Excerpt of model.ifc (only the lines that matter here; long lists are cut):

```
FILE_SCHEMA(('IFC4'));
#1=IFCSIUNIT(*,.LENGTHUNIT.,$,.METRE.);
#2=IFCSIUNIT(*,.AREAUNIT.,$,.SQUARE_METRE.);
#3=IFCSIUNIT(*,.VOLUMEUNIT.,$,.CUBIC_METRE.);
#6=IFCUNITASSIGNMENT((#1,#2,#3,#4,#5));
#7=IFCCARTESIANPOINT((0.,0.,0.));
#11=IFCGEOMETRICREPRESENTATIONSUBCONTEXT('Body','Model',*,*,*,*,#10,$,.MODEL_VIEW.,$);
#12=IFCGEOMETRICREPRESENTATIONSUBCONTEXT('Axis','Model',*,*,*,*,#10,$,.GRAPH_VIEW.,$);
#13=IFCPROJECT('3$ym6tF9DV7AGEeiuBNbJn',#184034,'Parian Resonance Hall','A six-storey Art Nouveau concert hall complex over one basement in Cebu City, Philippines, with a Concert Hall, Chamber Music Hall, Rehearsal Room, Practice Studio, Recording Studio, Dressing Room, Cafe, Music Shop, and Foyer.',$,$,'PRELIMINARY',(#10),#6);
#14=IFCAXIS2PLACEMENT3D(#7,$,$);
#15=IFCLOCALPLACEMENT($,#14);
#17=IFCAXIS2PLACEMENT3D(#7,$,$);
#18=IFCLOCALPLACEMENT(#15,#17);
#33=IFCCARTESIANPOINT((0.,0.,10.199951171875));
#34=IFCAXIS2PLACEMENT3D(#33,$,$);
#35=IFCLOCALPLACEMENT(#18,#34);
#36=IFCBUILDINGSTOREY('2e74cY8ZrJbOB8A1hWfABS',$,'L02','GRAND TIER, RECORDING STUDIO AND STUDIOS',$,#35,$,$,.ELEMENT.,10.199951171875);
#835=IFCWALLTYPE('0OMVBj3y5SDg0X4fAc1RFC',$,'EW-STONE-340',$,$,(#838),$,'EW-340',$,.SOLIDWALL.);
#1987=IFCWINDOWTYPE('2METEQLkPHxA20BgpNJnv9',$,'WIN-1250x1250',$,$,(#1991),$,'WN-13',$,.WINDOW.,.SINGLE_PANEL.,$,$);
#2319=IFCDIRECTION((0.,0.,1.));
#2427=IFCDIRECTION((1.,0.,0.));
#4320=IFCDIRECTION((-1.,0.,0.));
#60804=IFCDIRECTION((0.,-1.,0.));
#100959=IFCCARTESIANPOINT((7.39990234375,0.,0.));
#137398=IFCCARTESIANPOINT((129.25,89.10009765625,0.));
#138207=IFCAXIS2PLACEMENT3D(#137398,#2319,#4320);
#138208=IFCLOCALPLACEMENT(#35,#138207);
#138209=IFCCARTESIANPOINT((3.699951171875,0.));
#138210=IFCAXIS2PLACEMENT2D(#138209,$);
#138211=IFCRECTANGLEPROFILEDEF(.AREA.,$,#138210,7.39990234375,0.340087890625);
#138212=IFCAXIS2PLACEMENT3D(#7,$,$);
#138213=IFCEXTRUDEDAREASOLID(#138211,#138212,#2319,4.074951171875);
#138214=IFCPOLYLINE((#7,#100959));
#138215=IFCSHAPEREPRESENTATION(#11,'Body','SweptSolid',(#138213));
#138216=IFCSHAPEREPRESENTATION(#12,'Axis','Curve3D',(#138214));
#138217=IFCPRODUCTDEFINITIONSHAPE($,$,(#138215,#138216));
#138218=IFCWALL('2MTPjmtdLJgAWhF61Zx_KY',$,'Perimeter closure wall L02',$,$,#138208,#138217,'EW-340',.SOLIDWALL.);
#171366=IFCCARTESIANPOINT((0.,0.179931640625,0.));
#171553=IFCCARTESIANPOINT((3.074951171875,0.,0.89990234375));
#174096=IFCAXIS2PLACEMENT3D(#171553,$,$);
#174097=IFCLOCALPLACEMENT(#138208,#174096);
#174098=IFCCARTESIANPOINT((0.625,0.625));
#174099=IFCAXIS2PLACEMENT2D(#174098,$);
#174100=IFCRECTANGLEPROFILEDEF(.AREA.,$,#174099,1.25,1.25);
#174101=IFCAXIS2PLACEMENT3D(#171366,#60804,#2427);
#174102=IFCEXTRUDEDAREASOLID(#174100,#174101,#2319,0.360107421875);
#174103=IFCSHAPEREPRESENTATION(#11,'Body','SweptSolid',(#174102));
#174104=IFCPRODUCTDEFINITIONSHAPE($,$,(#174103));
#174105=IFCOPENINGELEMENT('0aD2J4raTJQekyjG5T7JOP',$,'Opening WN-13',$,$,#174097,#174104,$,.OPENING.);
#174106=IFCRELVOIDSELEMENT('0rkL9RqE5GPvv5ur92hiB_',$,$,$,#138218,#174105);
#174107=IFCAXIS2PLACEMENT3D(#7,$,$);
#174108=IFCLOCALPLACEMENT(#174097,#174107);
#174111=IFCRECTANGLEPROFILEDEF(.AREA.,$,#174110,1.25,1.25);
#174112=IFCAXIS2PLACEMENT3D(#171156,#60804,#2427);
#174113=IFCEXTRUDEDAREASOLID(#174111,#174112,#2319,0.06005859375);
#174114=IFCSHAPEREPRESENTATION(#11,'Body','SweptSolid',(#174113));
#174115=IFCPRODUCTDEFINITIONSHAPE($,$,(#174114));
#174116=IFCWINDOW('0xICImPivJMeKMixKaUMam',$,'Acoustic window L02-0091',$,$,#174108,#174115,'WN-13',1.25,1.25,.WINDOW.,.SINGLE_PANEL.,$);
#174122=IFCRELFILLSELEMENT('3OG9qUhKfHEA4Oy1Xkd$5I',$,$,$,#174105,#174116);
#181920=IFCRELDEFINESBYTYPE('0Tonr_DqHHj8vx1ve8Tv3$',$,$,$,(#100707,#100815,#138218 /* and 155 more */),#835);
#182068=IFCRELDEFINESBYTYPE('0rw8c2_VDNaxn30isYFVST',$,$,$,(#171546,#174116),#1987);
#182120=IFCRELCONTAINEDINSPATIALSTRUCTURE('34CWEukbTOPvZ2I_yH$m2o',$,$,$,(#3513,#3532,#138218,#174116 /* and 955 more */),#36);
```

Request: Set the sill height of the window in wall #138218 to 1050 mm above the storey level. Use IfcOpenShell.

```python
import numpy as np
import ifcopenshell
import ifcopenshell.api.geometry
import ifcopenshell.geom
import ifcopenshell.util.element
import ifcopenshell.util.placement
import ifcopenshell.util.shape
import ifcopenshell.util.unit

model = ifcopenshell.open("model.ifc")
unit_scale = ifcopenshell.util.unit.calculate_unit_scale(model)

window = model.by_guid("0xICImPivJMeKMixKaUMam")
opening = window.FillsVoids[0].RelatingOpeningElement
storey = ifcopenshell.util.element.get_container(window, ifc_class="IfcBuildingStorey")
level = ifcopenshell.util.placement.get_local_placement(storey.ObjectPlacement)[2, 3]

# The opening's origin need not be at the sill, so measure its lowest point.
shape = ifcopenshell.geom.create_shape(ifcopenshell.geom.settings(), opening)
bottom = ifcopenshell.util.shape.get_shape_bottom_elevation(shape, shape.geometry) / unit_scale
dz = level + 1.05 / unit_scale - bottom

shift = np.array([0.0, 0.0, dz])
# The window is placed relative to its opening, so it follows when the opening moves.
matrix = ifcopenshell.util.placement.get_local_placement(opening.ObjectPlacement)
matrix[:3, 3] += shift
ifcopenshell.api.geometry.edit_object_placement(
    model, product=opening, matrix=matrix, is_si=False, should_transform_children=True
)

print(f"moved by {dz * unit_scale:+.3f} m")

model.write("model_edited.ifc")
```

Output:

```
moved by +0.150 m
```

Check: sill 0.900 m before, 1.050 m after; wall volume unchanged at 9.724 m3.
